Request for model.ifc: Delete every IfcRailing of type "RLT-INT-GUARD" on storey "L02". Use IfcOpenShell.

First a look at what the model holds.

```python
import ifcopenshell
import ifcopenshell.util.element

model = ifcopenshell.open("model.ifc")
print(model.schema)
storey = next(s for s in model.by_type("IfcBuildingStorey") if s.Name == "L02")
railings = [e for e in ifcopenshell.util.element.get_decomposition(storey) if e.is_a("IfcRailing")]
seen = {}
for e in railings:
    element_type = ifcopenshell.util.element.get_type(e)
    name = element_type.Name if element_type not in (None, e) else None
    seen[name] = seen.get(name, 0) + 1
for name, count in sorted(seen.items(), key=str):
    print(count, "x", name)
```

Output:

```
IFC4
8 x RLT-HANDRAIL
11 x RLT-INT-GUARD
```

```python
import ifcopenshell
import ifcopenshell.api.root
import ifcopenshell.util.element

model = ifcopenshell.open("model.ifc")

storey = next(s for s in model.by_type("IfcBuildingStorey") if s.Name == "L02")
railings = [e for e in ifcopenshell.util.element.get_decomposition(storey) if e.is_a("IfcRailing")]
targets = [e for e in railings if (t := ifcopenshell.util.element.get_type(e)) not in (None, e) and t.Name == "RLT-INT-GUARD"]

for e in targets:
    ifcopenshell.api.root.remove_product(model, product=e)
print(len(targets), "removed")

model.write("model-out.ifc")
```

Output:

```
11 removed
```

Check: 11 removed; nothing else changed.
